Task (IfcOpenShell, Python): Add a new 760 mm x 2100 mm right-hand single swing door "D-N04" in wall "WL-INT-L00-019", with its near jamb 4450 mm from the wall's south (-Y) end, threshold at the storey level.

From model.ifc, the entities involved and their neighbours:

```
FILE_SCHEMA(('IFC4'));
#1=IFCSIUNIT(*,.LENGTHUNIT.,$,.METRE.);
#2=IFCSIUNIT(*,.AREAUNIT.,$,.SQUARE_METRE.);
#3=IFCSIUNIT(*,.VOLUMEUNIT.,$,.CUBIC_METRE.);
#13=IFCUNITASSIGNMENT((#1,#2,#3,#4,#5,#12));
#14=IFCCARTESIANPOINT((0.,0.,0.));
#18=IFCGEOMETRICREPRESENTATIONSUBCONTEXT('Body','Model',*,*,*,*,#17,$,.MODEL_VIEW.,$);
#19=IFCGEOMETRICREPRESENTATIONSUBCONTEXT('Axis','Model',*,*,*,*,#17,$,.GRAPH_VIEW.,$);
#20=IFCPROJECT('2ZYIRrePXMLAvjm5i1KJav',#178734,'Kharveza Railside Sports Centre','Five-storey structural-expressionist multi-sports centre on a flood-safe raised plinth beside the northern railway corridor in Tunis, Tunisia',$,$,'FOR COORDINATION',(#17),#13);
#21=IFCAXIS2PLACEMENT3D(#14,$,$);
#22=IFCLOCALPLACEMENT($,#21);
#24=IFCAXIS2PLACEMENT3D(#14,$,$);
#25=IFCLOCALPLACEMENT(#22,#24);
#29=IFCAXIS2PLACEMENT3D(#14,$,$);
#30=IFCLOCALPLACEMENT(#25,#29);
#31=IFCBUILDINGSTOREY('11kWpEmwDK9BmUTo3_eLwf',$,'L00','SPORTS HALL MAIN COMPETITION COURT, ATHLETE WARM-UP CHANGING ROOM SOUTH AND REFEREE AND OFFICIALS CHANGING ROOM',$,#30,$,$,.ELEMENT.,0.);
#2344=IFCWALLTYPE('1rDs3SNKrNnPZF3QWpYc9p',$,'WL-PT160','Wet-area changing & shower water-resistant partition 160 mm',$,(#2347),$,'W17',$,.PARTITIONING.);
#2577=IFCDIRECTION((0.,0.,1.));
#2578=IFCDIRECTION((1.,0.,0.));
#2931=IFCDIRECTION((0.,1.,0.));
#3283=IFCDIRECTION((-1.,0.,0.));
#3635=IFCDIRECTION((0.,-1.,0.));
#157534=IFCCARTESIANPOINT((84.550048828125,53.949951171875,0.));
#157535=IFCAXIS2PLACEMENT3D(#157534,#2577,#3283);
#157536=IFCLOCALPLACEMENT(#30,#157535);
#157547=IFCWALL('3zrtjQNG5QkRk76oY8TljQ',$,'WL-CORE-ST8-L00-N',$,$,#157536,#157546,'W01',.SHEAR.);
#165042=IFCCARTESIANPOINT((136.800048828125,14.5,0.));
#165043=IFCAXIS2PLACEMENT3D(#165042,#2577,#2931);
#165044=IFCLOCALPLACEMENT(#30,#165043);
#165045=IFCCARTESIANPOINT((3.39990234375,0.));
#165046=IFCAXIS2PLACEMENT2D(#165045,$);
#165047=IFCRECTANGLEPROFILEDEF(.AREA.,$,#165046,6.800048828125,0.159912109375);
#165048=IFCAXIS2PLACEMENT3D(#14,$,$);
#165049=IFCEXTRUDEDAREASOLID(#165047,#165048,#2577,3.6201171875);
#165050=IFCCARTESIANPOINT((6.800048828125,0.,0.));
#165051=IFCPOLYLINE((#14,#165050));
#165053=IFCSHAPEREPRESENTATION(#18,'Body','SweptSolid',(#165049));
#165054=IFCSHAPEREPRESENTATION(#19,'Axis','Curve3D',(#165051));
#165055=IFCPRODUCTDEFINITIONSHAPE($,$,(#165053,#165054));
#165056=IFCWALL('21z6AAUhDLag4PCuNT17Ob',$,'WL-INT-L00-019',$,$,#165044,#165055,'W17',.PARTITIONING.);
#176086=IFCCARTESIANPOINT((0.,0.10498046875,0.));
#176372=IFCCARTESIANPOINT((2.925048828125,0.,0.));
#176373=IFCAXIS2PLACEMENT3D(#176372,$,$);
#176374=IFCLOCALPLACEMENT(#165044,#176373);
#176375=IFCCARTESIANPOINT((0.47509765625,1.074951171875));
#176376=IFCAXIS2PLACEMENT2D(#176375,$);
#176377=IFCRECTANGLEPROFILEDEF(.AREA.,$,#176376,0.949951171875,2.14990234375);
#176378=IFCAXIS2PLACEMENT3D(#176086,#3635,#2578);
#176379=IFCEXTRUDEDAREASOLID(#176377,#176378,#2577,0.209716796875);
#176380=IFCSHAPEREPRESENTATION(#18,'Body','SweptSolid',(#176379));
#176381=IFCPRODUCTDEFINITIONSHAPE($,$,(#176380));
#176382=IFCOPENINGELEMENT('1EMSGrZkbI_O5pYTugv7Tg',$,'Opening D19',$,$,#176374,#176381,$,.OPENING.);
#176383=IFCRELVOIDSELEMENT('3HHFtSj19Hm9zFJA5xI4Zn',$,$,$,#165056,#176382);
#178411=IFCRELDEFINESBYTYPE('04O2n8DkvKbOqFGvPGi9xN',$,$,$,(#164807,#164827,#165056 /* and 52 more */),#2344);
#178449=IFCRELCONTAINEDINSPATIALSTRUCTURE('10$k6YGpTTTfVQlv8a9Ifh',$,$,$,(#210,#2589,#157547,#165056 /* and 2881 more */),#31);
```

```python
import numpy as np
import ifcopenshell
import ifcopenshell.api.feature
import ifcopenshell.api.geometry
import ifcopenshell.api.root
import ifcopenshell.api.spatial
import ifcopenshell.geom
import ifcopenshell.util.element
import ifcopenshell.util.placement
import ifcopenshell.util.representation
import ifcopenshell.util.shape
import ifcopenshell.util.unit

model = ifcopenshell.open("model.ifc")
unit_scale = ifcopenshell.util.unit.calculate_unit_scale(model)
settings = ifcopenshell.geom.settings()


def volume(element):
    """Net volume in cubic metres, openings subtracted."""
    shape = ifcopenshell.geom.create_shape(settings, element)
    return ifcopenshell.util.shape.get_volume(shape.geometry)


wall = model.by_guid("21z6AAUhDLag4PCuNT17Ob")
storey = ifcopenshell.util.element.get_container(wall, ifc_class="IfcBuildingStorey")
context = ifcopenshell.util.representation.get_context(model, "Model", "Body", "MODEL_VIEW")
before = volume(wall)

width, height, from_end, sill = 0.76, 2.1, 4.45, 0.0  # metres

# The wall runs along its own X axis, and the end named is its -X end.
wall_shape = ifcopenshell.geom.create_shape(settings, wall)
x, y, z = ifcopenshell.util.shape.get_vertices(wall_shape.geometry).T
start = x.min() + from_end
face, thickness = float(y.min()), float(y.max() - y.min())
wall_matrix = ifcopenshell.util.placement.get_local_placement(wall.ObjectPlacement)
level = ifcopenshell.util.placement.get_local_placement(storey.ObjectPlacement)[2, 3]


def in_wall(x, y):
    """Placement at x, y metres in the wall's axes, at sill height."""
    matrix = wall_matrix.copy()
    matrix[:, 3] = wall_matrix @ np.array([x / unit_scale, y / unit_scale, 0.0, 1.0])
    matrix[2, 3] = level + sill / unit_scale
    return matrix


# Opening: a box that overshoots both wall faces by 50 mm.
opening = ifcopenshell.api.root.create_entity(model, ifc_class="IfcOpeningElement", predefined_type="OPENING")
box = ifcopenshell.api.geometry.add_wall_representation(
    model, context=context, length=width, height=height, thickness=thickness + 0.1
)
ifcopenshell.api.geometry.assign_representation(model, product=opening, representation=box)
ifcopenshell.api.geometry.edit_object_placement(model, product=opening, matrix=in_wall(start, face - 0.05), is_si=False)
ifcopenshell.api.feature.add_feature(model, feature=opening, element=wall)

door = ifcopenshell.api.root.create_entity(model, ifc_class="IfcDoor", name="D-N04", predefined_type="DOOR")
door.OverallWidth, door.OverallHeight = width / unit_scale, height / unit_scale
door.OperationType = "SINGLE_SWING_RIGHT"
body = ifcopenshell.api.geometry.add_door_representation(
    model,
    context=context,
    overall_width=door.OverallWidth,
    overall_height=door.OverallHeight,
    operation_type="SINGLE_SWING_RIGHT",
    lining_properties={"LiningDepth": thickness / unit_scale, "ThresholdDepth": thickness / unit_scale},
)
ifcopenshell.api.geometry.assign_representation(model, product=door, representation=body)
ifcopenshell.api.spatial.assign_container(model, products=[door], relating_structure=storey)
ifcopenshell.api.feature.add_filling(model, opening=opening, element=door)

# The lining spans the wall, so the door starts at the wall face.
ifcopenshell.api.geometry.edit_object_placement(model, product=door, matrix=in_wall(start, face), is_si=False)

after = volume(wall)

print(f"wall volume {before:.3f} -> {after:.3f} m3")

model.write("model-out.ifc")
```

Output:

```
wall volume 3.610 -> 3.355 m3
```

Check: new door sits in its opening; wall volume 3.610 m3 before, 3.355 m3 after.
